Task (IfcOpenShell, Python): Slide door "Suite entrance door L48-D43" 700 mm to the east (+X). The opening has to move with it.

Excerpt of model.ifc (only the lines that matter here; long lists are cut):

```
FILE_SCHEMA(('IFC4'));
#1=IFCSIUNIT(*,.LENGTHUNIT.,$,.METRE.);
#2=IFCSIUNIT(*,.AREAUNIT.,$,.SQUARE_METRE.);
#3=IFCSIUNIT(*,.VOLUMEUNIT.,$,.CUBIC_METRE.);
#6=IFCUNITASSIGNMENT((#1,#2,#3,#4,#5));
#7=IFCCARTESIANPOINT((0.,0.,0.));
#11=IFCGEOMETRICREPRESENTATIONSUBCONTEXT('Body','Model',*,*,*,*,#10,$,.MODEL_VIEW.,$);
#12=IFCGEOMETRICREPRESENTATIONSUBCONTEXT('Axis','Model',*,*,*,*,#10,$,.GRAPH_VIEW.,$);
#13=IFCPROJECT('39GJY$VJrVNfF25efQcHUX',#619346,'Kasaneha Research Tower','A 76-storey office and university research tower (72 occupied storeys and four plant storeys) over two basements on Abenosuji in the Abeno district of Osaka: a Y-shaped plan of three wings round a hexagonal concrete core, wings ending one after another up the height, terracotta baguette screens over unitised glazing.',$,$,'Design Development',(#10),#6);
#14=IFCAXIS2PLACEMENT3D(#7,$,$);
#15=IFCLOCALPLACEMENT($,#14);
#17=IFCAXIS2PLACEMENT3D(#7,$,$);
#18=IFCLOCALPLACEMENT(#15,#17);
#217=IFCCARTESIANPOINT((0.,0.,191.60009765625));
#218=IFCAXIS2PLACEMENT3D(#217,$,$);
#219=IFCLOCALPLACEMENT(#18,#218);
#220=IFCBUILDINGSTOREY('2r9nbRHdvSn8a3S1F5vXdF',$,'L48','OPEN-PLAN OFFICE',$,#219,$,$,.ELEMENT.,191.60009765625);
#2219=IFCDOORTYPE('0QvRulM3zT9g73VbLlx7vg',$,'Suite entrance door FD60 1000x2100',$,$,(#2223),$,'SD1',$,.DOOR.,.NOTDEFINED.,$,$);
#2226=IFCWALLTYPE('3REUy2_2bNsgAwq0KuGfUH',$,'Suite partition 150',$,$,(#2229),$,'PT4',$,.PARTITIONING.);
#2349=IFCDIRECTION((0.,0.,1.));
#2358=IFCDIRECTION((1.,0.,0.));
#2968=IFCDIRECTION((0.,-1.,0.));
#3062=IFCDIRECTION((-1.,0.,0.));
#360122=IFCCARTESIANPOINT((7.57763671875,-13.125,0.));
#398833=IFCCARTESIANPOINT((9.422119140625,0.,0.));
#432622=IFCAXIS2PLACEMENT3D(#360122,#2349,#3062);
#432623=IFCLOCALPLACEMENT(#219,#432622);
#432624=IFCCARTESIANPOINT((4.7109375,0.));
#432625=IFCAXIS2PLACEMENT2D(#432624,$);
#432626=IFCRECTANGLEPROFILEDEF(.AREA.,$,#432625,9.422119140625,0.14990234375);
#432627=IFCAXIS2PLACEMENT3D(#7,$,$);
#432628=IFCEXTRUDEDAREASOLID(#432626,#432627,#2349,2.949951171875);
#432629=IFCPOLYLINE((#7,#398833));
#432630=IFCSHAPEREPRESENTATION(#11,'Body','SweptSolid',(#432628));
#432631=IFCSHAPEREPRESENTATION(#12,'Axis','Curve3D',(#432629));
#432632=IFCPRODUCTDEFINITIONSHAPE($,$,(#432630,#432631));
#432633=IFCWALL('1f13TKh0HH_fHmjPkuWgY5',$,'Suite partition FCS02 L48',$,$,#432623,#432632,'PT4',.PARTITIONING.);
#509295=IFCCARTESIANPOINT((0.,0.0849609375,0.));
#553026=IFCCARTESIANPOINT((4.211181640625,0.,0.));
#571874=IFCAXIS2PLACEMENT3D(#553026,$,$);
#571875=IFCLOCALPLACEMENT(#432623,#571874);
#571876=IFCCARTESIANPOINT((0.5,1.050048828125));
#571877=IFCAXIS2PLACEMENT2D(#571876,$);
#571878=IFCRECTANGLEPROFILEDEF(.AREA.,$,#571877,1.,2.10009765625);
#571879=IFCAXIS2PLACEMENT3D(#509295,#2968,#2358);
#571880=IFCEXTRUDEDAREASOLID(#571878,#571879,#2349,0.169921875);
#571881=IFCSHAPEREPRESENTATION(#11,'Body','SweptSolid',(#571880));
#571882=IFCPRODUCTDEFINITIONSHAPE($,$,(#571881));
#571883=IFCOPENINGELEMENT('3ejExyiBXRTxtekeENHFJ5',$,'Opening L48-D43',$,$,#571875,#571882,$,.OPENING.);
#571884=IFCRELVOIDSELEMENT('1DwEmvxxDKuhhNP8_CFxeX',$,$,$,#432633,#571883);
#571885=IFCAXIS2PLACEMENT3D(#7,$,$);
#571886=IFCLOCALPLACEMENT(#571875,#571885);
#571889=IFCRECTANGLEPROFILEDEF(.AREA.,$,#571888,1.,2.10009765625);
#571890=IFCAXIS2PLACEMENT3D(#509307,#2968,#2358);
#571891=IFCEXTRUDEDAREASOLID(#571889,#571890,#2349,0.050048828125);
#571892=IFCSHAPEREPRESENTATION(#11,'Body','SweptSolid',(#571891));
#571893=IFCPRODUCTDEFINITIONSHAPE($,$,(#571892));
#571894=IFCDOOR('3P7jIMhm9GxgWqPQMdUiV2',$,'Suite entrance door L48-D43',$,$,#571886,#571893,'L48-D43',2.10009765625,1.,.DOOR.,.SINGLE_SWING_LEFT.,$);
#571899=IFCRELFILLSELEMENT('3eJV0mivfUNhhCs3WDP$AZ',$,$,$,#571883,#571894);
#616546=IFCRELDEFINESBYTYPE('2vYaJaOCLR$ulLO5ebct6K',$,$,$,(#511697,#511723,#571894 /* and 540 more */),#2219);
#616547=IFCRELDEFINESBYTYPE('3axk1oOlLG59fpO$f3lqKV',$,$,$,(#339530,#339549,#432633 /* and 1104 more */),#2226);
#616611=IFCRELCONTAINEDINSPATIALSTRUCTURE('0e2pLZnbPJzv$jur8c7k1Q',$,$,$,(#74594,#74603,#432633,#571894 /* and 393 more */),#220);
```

```python
import ifcopenshell
import ifcopenshell.api.geometry
import ifcopenshell.util.placement
import ifcopenshell.util.unit

model = ifcopenshell.open("model.ifc")
unit_scale = ifcopenshell.util.unit.calculate_unit_scale(model)

door = model.by_guid("3P7jIMhm9GxgWqPQMdUiV2")
opening = door.FillsVoids[0].RelatingOpeningElement
wall = opening.VoidsElements[0].RelatingBuildingElement

wall_matrix = ifcopenshell.util.placement.get_local_placement(wall.ObjectPlacement)
shift = wall_matrix[:3, 0] * -0.7 / unit_scale
before = ifcopenshell.util.placement.get_local_placement(door.ObjectPlacement)[:3, 3].copy()

# The door is placed relative to its opening, so it follows when the opening moves.
matrix = ifcopenshell.util.placement.get_local_placement(opening.ObjectPlacement)
matrix[:3, 3] += shift
ifcopenshell.api.geometry.edit_object_placement(
    model, product=opening, matrix=matrix, is_si=False, should_transform_children=True
)

after = ifcopenshell.util.placement.get_local_placement(door.ObjectPlacement)[:3, 3]
print("door moved by", (after - before).round(3) + 0.0)

model.write("model-out.ifc")
```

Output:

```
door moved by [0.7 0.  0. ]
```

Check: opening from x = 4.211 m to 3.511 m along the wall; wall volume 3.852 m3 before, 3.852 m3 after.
